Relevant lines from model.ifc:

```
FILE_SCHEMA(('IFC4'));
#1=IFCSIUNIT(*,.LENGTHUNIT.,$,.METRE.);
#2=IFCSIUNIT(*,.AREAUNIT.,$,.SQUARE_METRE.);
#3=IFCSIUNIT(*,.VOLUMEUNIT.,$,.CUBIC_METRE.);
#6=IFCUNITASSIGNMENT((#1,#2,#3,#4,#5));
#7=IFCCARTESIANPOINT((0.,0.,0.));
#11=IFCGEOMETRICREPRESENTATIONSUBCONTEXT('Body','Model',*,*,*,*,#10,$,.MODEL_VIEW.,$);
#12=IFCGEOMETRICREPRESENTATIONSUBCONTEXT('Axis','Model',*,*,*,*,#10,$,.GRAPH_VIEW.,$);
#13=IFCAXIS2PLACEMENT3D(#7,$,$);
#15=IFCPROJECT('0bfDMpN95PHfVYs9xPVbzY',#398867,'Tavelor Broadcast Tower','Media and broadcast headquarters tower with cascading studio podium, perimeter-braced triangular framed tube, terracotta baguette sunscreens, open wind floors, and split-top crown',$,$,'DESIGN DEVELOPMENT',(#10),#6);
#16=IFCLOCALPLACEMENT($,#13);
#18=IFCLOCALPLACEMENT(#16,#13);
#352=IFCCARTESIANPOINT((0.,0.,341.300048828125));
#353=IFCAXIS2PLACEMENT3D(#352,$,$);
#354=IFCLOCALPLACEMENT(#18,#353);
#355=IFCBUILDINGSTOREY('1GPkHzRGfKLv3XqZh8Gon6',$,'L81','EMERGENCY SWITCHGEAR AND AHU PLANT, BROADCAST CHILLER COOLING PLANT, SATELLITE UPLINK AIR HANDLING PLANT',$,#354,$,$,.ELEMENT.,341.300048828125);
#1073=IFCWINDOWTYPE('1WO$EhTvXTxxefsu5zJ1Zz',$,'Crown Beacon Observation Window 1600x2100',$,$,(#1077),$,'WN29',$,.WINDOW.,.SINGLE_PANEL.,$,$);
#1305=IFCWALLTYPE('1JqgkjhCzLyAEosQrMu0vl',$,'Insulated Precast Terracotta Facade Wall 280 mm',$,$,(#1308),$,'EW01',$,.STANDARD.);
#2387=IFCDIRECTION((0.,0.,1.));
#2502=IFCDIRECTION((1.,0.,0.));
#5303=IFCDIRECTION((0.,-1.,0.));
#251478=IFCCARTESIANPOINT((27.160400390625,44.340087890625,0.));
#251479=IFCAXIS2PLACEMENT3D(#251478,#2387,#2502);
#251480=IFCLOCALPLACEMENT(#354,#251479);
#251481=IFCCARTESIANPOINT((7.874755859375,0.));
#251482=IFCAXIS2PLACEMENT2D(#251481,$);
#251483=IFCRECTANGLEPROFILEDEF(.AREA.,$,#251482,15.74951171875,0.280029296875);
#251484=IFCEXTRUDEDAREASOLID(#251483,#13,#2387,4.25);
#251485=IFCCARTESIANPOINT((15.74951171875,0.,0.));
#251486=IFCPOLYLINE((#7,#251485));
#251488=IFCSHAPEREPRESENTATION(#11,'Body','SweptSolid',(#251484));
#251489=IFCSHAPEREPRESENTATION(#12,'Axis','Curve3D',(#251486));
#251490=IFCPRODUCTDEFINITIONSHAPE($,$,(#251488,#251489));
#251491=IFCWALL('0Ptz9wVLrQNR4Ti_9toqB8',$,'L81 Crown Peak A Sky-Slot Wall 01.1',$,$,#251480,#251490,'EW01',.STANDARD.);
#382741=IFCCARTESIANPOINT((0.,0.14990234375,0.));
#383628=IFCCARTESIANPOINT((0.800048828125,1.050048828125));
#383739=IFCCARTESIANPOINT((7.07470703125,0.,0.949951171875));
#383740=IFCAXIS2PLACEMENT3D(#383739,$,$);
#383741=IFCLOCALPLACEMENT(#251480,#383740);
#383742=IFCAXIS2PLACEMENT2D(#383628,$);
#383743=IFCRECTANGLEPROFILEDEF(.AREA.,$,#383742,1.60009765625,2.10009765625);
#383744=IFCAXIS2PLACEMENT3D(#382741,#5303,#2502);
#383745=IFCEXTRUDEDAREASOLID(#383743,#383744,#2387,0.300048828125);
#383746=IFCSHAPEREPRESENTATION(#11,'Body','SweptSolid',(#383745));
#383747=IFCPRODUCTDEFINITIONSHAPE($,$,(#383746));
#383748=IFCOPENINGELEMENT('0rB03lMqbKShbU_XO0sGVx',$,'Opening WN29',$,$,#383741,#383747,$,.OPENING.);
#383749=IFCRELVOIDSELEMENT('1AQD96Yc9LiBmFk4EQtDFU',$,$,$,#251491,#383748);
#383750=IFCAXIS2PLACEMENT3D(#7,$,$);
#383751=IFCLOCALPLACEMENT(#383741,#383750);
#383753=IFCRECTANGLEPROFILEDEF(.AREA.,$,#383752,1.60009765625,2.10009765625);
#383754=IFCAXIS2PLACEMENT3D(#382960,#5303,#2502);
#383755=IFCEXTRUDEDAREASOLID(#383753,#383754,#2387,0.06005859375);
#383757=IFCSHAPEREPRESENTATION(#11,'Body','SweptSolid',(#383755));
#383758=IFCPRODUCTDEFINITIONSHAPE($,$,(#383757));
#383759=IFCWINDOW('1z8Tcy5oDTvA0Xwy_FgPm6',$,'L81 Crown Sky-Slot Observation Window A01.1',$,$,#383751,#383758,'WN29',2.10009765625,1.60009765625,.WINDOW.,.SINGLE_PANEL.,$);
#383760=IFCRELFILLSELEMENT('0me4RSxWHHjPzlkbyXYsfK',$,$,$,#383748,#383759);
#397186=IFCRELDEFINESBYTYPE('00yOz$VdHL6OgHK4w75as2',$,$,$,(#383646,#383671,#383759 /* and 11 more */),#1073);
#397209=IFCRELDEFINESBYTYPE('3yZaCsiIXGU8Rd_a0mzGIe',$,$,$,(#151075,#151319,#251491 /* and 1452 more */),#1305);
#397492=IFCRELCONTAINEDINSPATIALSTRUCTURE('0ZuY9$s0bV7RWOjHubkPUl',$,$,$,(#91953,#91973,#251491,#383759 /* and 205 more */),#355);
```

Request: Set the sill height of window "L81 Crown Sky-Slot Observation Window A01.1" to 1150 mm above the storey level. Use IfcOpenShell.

```python
import numpy as np
import ifcopenshell
import ifcopenshell.api.geometry
import ifcopenshell.geom
import ifcopenshell.util.element
import ifcopenshell.util.placement
import ifcopenshell.util.shape
import ifcopenshell.util.unit

model = ifcopenshell.open("model.ifc")
unit_scale = ifcopenshell.util.unit.calculate_unit_scale(model)

window = model.by_id(383759)
opening = window.FillsVoids[0].RelatingOpeningElement
storey = ifcopenshell.util.element.get_container(window, ifc_class="IfcBuildingStorey")
level = ifcopenshell.util.placement.get_local_placement(storey.ObjectPlacement)[2, 3]

# The opening's origin need not be at the sill, so measure its lowest point.
shape = ifcopenshell.geom.create_shape(ifcopenshell.geom.settings(), opening)
bottom = ifcopenshell.util.shape.get_shape_bottom_elevation(shape, shape.geometry) / unit_scale
dz = level + 1.15 - bottom

shift = np.array([0.0, 0.0, dz])
# The window is placed relative to its opening, so it follows when the opening moves.
matrix = ifcopenshell.util.placement.get_local_placement(opening.ObjectPlacement)
matrix[:3, 3] += shift
ifcopenshell.api.geometry.edit_object_placement(
    model, product=opening, matrix=matrix, is_si=False, should_transform_children=True
)

print(f"moved by {dz * unit_scale:+.3f} m")

model.write("model_edited.ifc")
```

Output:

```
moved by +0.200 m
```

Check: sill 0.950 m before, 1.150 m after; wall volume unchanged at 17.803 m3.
